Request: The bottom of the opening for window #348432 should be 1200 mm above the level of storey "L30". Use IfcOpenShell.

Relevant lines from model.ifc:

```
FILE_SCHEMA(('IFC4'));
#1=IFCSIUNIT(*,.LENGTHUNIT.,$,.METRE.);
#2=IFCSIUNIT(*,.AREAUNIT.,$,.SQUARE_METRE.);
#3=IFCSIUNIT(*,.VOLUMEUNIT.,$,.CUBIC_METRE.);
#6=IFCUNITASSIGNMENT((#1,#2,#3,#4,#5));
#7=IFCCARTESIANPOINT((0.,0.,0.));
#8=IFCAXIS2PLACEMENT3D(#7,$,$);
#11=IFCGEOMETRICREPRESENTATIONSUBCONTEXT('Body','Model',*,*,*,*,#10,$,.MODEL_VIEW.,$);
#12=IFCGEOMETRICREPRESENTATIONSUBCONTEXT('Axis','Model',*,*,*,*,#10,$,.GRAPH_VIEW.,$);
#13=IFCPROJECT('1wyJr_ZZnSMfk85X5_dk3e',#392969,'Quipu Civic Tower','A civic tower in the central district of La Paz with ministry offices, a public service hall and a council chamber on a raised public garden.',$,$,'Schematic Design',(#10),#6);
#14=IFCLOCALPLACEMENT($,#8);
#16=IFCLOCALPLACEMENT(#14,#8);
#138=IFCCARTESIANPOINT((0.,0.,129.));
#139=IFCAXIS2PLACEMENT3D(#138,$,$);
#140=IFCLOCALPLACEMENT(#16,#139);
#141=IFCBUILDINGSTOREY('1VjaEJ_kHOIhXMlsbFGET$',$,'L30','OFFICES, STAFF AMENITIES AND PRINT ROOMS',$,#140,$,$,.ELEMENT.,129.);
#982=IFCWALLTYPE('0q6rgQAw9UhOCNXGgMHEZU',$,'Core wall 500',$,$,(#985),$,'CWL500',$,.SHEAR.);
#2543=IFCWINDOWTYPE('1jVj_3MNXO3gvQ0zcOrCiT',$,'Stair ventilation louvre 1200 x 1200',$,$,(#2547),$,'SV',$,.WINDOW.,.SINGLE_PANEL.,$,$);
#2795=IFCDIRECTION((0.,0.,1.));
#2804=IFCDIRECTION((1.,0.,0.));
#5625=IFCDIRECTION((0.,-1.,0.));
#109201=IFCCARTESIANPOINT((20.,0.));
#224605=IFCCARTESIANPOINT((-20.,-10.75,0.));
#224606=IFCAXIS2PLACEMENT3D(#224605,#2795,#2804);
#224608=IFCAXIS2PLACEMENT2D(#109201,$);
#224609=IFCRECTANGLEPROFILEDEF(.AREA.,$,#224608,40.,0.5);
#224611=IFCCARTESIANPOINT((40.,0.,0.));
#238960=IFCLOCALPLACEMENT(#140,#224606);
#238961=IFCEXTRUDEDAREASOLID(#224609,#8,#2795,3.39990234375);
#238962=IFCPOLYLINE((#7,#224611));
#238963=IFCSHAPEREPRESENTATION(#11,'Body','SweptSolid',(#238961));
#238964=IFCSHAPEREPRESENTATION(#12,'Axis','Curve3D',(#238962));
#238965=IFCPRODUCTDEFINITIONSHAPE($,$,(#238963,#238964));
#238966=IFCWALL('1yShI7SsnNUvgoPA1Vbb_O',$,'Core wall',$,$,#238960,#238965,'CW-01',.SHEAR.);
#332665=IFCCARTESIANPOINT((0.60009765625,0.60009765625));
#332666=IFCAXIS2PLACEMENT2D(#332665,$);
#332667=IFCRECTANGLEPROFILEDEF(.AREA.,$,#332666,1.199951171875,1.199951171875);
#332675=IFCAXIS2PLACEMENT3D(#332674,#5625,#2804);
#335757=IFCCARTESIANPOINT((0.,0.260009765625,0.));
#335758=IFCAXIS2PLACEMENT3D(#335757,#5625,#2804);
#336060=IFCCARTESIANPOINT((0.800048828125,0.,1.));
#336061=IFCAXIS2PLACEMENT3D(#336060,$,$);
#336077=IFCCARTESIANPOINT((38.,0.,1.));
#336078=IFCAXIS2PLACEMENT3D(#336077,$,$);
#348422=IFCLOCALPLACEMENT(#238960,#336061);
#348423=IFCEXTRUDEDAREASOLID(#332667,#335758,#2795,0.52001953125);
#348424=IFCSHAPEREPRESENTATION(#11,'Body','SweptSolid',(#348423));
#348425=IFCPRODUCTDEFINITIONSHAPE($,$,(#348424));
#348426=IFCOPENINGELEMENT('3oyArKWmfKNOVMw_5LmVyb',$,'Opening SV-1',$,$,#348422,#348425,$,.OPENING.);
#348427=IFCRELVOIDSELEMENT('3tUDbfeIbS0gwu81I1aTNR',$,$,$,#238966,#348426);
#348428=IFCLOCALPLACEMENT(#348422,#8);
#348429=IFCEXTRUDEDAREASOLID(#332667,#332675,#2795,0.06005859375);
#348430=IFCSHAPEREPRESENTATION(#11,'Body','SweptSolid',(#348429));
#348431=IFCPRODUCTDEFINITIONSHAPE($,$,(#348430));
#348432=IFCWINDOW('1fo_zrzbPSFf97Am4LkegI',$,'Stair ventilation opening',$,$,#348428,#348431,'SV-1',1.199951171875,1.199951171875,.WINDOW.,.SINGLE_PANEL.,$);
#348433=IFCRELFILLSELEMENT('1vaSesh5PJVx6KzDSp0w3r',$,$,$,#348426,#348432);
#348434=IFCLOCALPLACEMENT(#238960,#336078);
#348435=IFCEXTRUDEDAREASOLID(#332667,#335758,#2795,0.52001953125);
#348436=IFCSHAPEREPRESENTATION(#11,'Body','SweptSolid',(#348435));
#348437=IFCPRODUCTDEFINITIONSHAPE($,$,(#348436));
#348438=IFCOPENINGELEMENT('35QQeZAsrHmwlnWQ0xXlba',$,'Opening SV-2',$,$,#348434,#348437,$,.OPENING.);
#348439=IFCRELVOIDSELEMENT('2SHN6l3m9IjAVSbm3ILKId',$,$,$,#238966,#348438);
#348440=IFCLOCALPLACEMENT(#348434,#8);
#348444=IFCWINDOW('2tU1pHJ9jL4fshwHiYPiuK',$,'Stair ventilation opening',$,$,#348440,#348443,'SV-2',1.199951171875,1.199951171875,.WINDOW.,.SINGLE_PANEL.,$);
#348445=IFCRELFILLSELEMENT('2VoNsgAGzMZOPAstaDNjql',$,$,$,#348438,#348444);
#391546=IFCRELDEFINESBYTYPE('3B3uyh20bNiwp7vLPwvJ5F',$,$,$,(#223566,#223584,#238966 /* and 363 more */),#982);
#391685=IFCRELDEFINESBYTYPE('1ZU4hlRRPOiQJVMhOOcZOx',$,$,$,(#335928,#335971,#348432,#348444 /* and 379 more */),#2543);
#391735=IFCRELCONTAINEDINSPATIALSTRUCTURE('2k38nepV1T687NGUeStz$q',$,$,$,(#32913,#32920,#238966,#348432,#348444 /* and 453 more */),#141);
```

```python
import numpy as np
import ifcopenshell
import ifcopenshell.api.geometry
import ifcopenshell.geom
import ifcopenshell.util.element
import ifcopenshell.util.placement
import ifcopenshell.util.shape
import ifcopenshell.util.unit

model = ifcopenshell.open("model.ifc")
unit_scale = ifcopenshell.util.unit.calculate_unit_scale(model)

window = model.by_guid("1fo_zrzbPSFf97Am4LkegI")
opening = window.FillsVoids[0].RelatingOpeningElement
storey = ifcopenshell.util.element.get_container(window, ifc_class="IfcBuildingStorey")
level = ifcopenshell.util.placement.get_local_placement(storey.ObjectPlacement)[2, 3]

# The opening's origin need not be at the sill, so measure its lowest point.
shape = ifcopenshell.geom.create_shape(ifcopenshell.geom.settings(), opening)
bottom = ifcopenshell.util.shape.get_shape_bottom_elevation(shape, shape.geometry) / unit_scale
dz = level + 1.2 - bottom

shift = np.array([0.0, 0.0, dz])
# The window is placed relative to its opening, so it follows when the opening moves.
matrix = ifcopenshell.util.placement.get_local_placement(opening.ObjectPlacement)
matrix[:3, 3] += shift
ifcopenshell.api.geometry.edit_object_placement(
    model, product=opening, matrix=matrix, is_si=False, should_transform_children=True
)

print(f"moved by {dz * unit_scale:+.3f} m")

model.write("model_edited.ifc")
```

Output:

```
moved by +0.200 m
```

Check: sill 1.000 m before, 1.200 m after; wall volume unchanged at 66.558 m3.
